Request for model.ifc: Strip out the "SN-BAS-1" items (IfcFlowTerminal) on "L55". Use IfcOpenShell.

First a look at what the model holds.

```python
import ifcopenshell
import ifcopenshell.util.element

model = ifcopenshell.open("model.ifc")
print(model.schema)
storey = next(s for s in model.by_type("IfcBuildingStorey") if s.Name == "L55")
terminals = [e for e in ifcopenshell.util.element.get_decomposition(storey) if e.is_a("IfcFlowTerminal")]
seen = {}
for e in terminals:
    element_type = ifcopenshell.util.element.get_type(e)
    name = element_type.Name if element_type not in (None, e) else None
    seen[name] = seen.get(name, 0) + 1
for name, count in sorted(seen.items(), key=str):
    print(count, "x", name)
```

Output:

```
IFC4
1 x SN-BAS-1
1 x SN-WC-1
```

```python
import ifcopenshell
import ifcopenshell.api.root
import ifcopenshell.util.element

model = ifcopenshell.open("model.ifc")

storey = next(s for s in model.by_type("IfcBuildingStorey") if s.Name == "L55")
terminals = [e for e in ifcopenshell.util.element.get_decomposition(storey) if e.is_a("IfcFlowTerminal")]
targets = [e for e in terminals if (t := ifcopenshell.util.element.get_type(e)) not in (None, e) and t.Name == "SN-BAS-1"]

for e in targets:
    ifcopenshell.api.root.remove_product(model, product=e)
print(len(targets), "removed")

model.write("model_updated.ifc")
```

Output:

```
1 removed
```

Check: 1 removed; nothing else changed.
